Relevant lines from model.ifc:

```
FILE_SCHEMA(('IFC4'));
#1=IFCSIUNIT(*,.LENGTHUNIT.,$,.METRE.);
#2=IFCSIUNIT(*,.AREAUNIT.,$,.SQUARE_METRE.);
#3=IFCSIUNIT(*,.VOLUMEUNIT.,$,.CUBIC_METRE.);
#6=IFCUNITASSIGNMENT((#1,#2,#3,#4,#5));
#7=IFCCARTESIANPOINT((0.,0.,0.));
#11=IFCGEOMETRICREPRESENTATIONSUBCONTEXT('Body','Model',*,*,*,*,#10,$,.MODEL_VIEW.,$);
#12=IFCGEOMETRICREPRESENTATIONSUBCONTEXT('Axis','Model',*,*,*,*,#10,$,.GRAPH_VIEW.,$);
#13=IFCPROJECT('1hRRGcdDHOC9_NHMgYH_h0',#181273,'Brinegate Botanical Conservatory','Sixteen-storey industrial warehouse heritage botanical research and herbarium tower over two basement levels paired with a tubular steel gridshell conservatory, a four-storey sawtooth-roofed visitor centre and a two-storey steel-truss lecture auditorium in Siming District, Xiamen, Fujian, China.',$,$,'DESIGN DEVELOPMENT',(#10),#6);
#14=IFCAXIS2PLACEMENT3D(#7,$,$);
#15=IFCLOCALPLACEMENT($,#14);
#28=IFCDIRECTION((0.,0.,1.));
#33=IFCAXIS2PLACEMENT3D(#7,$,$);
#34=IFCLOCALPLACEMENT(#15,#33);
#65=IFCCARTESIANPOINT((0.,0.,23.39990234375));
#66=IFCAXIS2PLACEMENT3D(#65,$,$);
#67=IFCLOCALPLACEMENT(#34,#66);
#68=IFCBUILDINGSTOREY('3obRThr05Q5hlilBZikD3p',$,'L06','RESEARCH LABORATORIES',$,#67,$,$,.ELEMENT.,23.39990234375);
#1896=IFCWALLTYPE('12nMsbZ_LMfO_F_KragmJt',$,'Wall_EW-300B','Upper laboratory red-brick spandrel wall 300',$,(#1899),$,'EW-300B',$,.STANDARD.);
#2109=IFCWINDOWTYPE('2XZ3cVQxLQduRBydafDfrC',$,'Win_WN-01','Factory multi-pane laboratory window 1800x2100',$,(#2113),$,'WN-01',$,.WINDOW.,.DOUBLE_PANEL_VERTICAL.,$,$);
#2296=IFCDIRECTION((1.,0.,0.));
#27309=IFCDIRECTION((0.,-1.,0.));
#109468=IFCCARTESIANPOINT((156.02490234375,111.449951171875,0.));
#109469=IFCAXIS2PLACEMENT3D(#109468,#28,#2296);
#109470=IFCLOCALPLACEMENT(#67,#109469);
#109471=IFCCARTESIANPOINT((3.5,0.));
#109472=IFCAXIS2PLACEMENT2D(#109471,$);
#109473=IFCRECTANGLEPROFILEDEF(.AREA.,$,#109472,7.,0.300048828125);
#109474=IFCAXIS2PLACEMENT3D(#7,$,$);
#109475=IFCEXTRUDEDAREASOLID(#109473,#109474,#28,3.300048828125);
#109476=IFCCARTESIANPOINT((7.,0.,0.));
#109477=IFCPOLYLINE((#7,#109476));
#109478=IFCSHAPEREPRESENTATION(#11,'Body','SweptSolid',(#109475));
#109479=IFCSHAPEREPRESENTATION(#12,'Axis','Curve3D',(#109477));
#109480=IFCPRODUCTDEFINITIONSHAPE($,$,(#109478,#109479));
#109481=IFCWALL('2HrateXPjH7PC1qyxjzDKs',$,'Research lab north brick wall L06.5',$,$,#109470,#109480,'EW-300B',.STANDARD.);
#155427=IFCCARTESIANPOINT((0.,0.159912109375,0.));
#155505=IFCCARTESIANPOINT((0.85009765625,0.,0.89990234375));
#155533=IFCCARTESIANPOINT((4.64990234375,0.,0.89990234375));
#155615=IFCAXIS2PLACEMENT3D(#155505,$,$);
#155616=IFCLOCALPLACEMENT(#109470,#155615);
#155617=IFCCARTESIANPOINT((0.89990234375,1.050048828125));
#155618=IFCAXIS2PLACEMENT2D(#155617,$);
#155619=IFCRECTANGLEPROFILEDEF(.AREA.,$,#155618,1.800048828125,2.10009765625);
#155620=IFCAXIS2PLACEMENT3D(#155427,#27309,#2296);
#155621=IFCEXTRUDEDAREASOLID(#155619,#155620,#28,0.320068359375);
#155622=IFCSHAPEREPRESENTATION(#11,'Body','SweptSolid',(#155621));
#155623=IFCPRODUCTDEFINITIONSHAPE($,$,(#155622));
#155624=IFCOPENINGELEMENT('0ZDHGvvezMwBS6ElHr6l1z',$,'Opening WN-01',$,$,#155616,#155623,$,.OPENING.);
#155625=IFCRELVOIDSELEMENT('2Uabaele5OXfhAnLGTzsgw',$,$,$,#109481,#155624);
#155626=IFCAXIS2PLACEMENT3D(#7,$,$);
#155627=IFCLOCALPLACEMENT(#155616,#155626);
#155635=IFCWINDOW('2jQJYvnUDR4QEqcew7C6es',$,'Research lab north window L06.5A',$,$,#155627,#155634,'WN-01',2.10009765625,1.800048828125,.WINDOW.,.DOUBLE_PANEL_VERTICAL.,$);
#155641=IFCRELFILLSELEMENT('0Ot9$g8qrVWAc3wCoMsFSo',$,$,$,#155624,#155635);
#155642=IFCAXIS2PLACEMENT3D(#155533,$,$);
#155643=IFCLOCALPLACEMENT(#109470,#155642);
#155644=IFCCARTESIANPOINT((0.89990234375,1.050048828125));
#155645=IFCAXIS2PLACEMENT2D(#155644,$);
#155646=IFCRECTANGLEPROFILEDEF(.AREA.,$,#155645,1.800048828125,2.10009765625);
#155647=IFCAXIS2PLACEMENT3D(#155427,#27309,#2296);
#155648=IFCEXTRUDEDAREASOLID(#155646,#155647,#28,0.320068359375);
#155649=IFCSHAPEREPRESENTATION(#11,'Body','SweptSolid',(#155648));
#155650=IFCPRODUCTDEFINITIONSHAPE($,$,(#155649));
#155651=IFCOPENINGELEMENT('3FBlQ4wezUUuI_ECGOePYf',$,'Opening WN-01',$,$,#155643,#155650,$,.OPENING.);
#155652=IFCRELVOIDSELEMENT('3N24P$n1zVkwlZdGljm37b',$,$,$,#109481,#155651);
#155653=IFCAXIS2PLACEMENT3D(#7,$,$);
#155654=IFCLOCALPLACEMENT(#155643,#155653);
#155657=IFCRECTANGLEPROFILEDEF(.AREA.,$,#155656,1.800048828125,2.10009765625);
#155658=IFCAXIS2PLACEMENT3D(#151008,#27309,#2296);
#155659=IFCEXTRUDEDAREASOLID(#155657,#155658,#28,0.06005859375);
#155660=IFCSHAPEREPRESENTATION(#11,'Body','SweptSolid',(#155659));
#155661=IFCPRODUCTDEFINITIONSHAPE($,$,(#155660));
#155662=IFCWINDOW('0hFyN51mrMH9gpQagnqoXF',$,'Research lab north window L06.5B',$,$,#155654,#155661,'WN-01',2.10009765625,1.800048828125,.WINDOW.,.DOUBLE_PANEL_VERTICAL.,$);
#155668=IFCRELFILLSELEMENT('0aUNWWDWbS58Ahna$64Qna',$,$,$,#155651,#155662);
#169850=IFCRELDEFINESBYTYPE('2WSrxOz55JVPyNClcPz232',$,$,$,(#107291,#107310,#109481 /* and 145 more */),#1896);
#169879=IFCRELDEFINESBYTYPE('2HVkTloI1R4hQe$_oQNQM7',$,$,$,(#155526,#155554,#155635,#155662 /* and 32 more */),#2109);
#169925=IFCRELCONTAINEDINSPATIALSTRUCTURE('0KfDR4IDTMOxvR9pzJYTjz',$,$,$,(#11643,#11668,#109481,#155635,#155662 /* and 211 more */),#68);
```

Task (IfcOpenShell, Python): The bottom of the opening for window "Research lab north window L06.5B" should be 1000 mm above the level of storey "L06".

```python
import numpy as np
import ifcopenshell
import ifcopenshell.api.geometry
import ifcopenshell.geom
import ifcopenshell.util.element
import ifcopenshell.util.placement
import ifcopenshell.util.shape
import ifcopenshell.util.unit

model = ifcopenshell.open("model.ifc")
unit_scale = ifcopenshell.util.unit.calculate_unit_scale(model)

window = model.by_guid("0hFyN51mrMH9gpQagnqoXF")
opening = window.FillsVoids[0].RelatingOpeningElement
storey = ifcopenshell.util.element.get_container(window, ifc_class="IfcBuildingStorey")
level = ifcopenshell.util.placement.get_local_placement(storey.ObjectPlacement)[2, 3]

# The opening's origin need not be at the sill, so measure its lowest point.
shape = ifcopenshell.geom.create_shape(ifcopenshell.geom.settings(), opening)
bottom = ifcopenshell.util.shape.get_shape_bottom_elevation(shape, shape.geometry) / unit_scale
dz = level + 1.0 - bottom

shift = np.array([0.0, 0.0, dz])
# The window is placed relative to its opening, so it follows when the opening moves.
matrix = ifcopenshell.util.placement.get_local_placement(opening.ObjectPlacement)
matrix[:3, 3] += shift
ifcopenshell.api.geometry.edit_object_placement(
    model, product=opening, matrix=matrix, is_si=False, should_transform_children=True
)

print(f"moved by {dz * unit_scale:+.3f} m")

model.write("model_rev.ifc")
```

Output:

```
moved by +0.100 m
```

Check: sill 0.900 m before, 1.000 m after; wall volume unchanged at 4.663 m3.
